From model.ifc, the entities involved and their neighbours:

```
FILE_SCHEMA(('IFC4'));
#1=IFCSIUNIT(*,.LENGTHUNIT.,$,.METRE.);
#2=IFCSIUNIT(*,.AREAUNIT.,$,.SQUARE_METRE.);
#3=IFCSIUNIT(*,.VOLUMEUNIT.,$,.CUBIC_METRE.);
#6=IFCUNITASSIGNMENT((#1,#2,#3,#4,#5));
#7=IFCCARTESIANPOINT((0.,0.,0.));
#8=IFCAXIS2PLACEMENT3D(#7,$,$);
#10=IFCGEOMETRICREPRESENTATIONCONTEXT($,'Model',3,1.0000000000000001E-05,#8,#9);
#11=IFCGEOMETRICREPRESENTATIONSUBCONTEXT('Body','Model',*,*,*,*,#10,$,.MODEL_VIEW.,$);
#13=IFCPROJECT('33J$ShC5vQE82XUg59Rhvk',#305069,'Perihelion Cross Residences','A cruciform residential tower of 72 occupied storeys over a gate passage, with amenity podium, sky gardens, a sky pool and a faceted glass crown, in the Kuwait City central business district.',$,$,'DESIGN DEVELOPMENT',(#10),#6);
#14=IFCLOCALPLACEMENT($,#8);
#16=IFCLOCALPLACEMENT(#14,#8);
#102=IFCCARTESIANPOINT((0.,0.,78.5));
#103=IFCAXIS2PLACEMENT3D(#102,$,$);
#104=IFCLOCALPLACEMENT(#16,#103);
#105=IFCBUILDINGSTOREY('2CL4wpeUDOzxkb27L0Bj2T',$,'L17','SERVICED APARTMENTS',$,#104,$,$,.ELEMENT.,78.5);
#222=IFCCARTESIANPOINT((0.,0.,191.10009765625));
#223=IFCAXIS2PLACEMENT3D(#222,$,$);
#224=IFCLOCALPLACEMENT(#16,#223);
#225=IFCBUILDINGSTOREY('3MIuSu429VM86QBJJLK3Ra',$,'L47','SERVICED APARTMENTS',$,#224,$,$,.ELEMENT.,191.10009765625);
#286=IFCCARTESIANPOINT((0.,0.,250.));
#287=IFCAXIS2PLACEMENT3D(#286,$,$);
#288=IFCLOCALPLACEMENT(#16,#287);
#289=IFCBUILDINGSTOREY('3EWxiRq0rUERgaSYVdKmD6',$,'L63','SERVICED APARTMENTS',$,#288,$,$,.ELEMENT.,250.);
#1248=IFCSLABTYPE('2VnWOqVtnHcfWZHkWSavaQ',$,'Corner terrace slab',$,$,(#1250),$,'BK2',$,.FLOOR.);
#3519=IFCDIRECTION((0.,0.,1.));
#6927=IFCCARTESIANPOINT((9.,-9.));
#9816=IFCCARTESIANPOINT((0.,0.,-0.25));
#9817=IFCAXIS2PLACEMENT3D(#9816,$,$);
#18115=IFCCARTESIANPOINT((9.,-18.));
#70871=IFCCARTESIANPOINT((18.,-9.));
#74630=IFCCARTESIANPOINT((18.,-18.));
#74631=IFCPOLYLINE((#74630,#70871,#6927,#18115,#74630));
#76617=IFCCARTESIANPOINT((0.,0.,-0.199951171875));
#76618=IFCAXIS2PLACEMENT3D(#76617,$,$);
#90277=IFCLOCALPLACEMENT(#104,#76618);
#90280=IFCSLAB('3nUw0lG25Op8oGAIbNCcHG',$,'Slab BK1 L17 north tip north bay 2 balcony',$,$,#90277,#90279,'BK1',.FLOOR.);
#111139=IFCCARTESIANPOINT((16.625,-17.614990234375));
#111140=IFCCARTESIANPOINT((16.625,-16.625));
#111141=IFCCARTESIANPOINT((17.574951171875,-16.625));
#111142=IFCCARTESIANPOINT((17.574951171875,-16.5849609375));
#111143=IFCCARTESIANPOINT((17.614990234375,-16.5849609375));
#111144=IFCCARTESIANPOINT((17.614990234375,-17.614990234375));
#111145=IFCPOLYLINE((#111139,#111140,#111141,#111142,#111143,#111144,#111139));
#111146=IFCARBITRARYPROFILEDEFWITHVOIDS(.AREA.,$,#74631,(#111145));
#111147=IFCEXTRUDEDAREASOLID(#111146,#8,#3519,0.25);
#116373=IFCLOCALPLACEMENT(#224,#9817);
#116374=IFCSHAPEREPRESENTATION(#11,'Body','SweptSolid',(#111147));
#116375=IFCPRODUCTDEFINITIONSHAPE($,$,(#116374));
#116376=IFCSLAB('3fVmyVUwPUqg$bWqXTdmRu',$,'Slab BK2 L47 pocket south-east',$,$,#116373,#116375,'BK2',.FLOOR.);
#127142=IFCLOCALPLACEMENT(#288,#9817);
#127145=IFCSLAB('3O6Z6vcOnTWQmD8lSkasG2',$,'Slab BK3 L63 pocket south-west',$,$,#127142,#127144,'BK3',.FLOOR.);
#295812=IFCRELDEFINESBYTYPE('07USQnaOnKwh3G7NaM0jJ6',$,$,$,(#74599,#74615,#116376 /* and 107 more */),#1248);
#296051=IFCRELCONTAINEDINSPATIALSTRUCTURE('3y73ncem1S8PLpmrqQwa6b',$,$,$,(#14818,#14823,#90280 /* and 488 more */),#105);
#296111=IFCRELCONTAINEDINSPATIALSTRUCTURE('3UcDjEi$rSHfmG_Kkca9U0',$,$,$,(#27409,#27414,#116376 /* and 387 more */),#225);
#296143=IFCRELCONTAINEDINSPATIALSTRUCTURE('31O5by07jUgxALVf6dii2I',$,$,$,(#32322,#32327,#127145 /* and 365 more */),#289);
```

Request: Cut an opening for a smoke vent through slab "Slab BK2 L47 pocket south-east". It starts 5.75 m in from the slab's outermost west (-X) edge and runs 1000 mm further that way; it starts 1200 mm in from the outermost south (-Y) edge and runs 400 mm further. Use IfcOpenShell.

```python
import numpy as np
import ifcopenshell
import ifcopenshell.api.feature
import ifcopenshell.api.geometry
import ifcopenshell.api.root
import ifcopenshell.geom
import ifcopenshell.util.placement
import ifcopenshell.util.representation
import ifcopenshell.util.shape
import ifcopenshell.util.unit

model = ifcopenshell.open("model.ifc")
unit_scale = ifcopenshell.util.unit.calculate_unit_scale(model)
settings = ifcopenshell.geom.settings()


def volume(element):
    """Net volume in cubic metres, openings subtracted."""
    shape = ifcopenshell.geom.create_shape(settings, element)
    return ifcopenshell.util.shape.get_volume(shape.geometry)


slab = model.by_id(116376)
before = volume(slab)

# Extent in the slab's own axes, in metres. The edges named are its -X and -Y sides.
slab_shape = ifcopenshell.geom.create_shape(settings, slab)
vertices = ifcopenshell.util.shape.get_vertices(slab_shape.geometry)
x_min, y_min, bottom = vertices.min(axis=0)
top = vertices[:, 2].max()

opening = ifcopenshell.api.root.create_entity(model, ifc_class="IfcOpeningElement", name="Smoke vent opening", predefined_type="OPENING")
context = ifcopenshell.util.representation.get_context(model, "Model", "Body", "MODEL_VIEW")
width, depth = 1, 0.4
outline = [(0.0, 0.0), (width, 0.0), (width, depth), (0.0, depth), (0.0, 0.0)]
# Overshoot both faces by 50 mm so the cut is clean.
shape = ifcopenshell.api.geometry.add_slab_representation(
    model, context=context, depth=top - bottom + 0.1, polyline=outline
)
ifcopenshell.api.geometry.assign_representation(model, product=opening, representation=shape)

matrix = ifcopenshell.util.placement.get_local_placement(slab.ObjectPlacement)
matrix[:, 3] = matrix @ np.append(np.array([x_min + 5.75, y_min + 1.2, bottom - 0.05]) / unit_scale, 1.0)
ifcopenshell.api.geometry.edit_object_placement(model, product=opening, matrix=matrix, is_si=False)
ifcopenshell.api.feature.add_feature(model, feature=opening, element=slab)

after = volume(slab)

print(f"slab volume {before:.3f} -> {after:.3f} m3")

model.write("model_rev.ifc")
```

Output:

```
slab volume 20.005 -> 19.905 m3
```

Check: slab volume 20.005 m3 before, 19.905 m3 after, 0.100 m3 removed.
